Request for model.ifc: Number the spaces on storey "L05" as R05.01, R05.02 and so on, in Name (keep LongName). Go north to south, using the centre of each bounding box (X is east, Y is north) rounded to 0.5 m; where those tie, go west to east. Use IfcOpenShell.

First a look at what the model holds.

```python
import ifcopenshell
import ifcopenshell.util.element
import ifcopenshell.util.placement

model = ifcopenshell.open("model.ifc")
print(model.schema)
storey = next(s for s in model.by_type("IfcBuildingStorey") if s.Name == "L05")
spaces = [e for e in ifcopenshell.util.element.get_decomposition(storey) if e.is_a("IfcSpace")]
for e in sorted(spaces, key=lambda e: e.id()):
    origin = ifcopenshell.util.placement.get_local_placement(e.ObjectPlacement)[:3, 3]
    print(e.id(), e.Name, e.LongName, origin.round(2) + 0.0, sep=" | ")
```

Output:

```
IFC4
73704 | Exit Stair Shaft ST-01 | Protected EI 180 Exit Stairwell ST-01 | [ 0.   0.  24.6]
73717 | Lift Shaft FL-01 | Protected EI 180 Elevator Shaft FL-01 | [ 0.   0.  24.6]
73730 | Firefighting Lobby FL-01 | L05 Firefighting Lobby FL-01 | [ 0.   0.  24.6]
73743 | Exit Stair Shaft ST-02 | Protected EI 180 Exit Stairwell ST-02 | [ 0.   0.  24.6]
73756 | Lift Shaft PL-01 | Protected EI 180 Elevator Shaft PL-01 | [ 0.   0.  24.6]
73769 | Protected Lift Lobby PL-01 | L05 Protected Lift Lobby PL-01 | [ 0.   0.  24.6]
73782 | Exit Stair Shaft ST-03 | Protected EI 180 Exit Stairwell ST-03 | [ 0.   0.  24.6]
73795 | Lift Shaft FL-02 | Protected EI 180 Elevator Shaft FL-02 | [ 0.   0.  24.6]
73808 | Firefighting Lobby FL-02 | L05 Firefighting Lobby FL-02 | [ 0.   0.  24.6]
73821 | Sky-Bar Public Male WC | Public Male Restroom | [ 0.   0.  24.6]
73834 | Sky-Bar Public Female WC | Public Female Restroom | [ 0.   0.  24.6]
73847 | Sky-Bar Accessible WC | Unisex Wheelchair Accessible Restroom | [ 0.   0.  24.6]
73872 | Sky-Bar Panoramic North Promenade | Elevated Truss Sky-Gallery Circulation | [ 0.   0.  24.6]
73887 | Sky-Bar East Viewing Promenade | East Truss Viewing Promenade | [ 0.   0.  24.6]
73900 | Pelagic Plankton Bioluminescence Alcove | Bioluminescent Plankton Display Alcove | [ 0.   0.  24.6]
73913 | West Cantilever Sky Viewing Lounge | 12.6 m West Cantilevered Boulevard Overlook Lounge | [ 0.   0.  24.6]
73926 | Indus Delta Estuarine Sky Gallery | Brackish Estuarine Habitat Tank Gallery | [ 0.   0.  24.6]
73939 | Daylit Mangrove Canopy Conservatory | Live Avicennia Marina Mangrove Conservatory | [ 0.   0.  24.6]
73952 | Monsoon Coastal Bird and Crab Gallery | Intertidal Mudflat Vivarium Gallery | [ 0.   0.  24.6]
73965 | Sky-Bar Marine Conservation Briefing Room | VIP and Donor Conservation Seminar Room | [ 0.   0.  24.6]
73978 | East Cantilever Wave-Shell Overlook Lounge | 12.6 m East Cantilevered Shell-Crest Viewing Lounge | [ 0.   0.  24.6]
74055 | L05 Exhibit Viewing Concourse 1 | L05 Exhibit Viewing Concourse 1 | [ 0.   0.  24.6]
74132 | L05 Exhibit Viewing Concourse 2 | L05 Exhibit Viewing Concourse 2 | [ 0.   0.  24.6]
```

```python
import ifcopenshell
import ifcopenshell.geom
import ifcopenshell.util.element
import ifcopenshell.util.shape

model = ifcopenshell.open("model.ifc")
settings = ifcopenshell.geom.settings()
settings.set("use-world-coords", True)


def centre(element):
    shape = ifcopenshell.geom.create_shape(settings, element)
    return ifcopenshell.util.shape.get_bbox_centroid(shape.geometry)


storey = next(s for s in model.by_type("IfcBuildingStorey") if s.Name == "L05")
spaces = [e for e in ifcopenshell.util.element.get_decomposition(storey) if e.is_a("IfcSpace")]

# Insertion points can sit at a corner or the storey origin, so sort by the geometry (in metres).
centres = {e: centre(e) for e in spaces}
spaces.sort(key=lambda e: (-round(centres[e][1] / 0.5), centres[e][0]))

for i, e in enumerate(spaces, start=1):
    number = f"R05.{i:02d}"
    e.Name = number
    print(e.id(), number)

model.write("model_edited.ifc")
```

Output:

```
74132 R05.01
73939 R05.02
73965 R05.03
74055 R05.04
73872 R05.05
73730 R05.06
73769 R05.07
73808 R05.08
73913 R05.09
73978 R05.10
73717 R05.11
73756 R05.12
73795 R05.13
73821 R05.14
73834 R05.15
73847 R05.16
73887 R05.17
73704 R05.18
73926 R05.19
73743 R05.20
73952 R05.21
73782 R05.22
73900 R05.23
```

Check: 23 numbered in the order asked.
